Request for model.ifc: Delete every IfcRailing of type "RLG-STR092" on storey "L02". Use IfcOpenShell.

First a look at what the model holds.

```python
import ifcopenshell
import ifcopenshell.util.element

model = ifcopenshell.open("model.ifc")
print(model.schema)
storey = next(s for s in model.by_type("IfcBuildingStorey") if s.Name == "L02")
railings = [e for e in ifcopenshell.util.element.get_decomposition(storey) if e.is_a("IfcRailing")]
seen = {}
for e in railings:
    element_type = ifcopenshell.util.element.get_type(e)
    name = element_type.Name if element_type not in (None, e) else None
    seen[name] = seen.get(name, 0) + 1
for name, count in sorted(seen.items(), key=str):
    print(count, "x", name)
```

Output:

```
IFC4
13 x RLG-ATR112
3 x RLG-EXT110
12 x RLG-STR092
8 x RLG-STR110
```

```python
import ifcopenshell
import ifcopenshell.api.root
import ifcopenshell.util.element

model = ifcopenshell.open("model.ifc")

storey = next(s for s in model.by_type("IfcBuildingStorey") if s.Name == "L02")
railings = [e for e in ifcopenshell.util.element.get_decomposition(storey) if e.is_a("IfcRailing")]
targets = [e for e in railings if (t := ifcopenshell.util.element.get_type(e)) not in (None, e) and t.Name == "RLG-STR092"]

for e in targets:
    ifcopenshell.api.root.remove_product(model, product=e)
print(len(targets), "removed")

model.write("model_edited.ifc")
```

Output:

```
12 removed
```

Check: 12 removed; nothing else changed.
